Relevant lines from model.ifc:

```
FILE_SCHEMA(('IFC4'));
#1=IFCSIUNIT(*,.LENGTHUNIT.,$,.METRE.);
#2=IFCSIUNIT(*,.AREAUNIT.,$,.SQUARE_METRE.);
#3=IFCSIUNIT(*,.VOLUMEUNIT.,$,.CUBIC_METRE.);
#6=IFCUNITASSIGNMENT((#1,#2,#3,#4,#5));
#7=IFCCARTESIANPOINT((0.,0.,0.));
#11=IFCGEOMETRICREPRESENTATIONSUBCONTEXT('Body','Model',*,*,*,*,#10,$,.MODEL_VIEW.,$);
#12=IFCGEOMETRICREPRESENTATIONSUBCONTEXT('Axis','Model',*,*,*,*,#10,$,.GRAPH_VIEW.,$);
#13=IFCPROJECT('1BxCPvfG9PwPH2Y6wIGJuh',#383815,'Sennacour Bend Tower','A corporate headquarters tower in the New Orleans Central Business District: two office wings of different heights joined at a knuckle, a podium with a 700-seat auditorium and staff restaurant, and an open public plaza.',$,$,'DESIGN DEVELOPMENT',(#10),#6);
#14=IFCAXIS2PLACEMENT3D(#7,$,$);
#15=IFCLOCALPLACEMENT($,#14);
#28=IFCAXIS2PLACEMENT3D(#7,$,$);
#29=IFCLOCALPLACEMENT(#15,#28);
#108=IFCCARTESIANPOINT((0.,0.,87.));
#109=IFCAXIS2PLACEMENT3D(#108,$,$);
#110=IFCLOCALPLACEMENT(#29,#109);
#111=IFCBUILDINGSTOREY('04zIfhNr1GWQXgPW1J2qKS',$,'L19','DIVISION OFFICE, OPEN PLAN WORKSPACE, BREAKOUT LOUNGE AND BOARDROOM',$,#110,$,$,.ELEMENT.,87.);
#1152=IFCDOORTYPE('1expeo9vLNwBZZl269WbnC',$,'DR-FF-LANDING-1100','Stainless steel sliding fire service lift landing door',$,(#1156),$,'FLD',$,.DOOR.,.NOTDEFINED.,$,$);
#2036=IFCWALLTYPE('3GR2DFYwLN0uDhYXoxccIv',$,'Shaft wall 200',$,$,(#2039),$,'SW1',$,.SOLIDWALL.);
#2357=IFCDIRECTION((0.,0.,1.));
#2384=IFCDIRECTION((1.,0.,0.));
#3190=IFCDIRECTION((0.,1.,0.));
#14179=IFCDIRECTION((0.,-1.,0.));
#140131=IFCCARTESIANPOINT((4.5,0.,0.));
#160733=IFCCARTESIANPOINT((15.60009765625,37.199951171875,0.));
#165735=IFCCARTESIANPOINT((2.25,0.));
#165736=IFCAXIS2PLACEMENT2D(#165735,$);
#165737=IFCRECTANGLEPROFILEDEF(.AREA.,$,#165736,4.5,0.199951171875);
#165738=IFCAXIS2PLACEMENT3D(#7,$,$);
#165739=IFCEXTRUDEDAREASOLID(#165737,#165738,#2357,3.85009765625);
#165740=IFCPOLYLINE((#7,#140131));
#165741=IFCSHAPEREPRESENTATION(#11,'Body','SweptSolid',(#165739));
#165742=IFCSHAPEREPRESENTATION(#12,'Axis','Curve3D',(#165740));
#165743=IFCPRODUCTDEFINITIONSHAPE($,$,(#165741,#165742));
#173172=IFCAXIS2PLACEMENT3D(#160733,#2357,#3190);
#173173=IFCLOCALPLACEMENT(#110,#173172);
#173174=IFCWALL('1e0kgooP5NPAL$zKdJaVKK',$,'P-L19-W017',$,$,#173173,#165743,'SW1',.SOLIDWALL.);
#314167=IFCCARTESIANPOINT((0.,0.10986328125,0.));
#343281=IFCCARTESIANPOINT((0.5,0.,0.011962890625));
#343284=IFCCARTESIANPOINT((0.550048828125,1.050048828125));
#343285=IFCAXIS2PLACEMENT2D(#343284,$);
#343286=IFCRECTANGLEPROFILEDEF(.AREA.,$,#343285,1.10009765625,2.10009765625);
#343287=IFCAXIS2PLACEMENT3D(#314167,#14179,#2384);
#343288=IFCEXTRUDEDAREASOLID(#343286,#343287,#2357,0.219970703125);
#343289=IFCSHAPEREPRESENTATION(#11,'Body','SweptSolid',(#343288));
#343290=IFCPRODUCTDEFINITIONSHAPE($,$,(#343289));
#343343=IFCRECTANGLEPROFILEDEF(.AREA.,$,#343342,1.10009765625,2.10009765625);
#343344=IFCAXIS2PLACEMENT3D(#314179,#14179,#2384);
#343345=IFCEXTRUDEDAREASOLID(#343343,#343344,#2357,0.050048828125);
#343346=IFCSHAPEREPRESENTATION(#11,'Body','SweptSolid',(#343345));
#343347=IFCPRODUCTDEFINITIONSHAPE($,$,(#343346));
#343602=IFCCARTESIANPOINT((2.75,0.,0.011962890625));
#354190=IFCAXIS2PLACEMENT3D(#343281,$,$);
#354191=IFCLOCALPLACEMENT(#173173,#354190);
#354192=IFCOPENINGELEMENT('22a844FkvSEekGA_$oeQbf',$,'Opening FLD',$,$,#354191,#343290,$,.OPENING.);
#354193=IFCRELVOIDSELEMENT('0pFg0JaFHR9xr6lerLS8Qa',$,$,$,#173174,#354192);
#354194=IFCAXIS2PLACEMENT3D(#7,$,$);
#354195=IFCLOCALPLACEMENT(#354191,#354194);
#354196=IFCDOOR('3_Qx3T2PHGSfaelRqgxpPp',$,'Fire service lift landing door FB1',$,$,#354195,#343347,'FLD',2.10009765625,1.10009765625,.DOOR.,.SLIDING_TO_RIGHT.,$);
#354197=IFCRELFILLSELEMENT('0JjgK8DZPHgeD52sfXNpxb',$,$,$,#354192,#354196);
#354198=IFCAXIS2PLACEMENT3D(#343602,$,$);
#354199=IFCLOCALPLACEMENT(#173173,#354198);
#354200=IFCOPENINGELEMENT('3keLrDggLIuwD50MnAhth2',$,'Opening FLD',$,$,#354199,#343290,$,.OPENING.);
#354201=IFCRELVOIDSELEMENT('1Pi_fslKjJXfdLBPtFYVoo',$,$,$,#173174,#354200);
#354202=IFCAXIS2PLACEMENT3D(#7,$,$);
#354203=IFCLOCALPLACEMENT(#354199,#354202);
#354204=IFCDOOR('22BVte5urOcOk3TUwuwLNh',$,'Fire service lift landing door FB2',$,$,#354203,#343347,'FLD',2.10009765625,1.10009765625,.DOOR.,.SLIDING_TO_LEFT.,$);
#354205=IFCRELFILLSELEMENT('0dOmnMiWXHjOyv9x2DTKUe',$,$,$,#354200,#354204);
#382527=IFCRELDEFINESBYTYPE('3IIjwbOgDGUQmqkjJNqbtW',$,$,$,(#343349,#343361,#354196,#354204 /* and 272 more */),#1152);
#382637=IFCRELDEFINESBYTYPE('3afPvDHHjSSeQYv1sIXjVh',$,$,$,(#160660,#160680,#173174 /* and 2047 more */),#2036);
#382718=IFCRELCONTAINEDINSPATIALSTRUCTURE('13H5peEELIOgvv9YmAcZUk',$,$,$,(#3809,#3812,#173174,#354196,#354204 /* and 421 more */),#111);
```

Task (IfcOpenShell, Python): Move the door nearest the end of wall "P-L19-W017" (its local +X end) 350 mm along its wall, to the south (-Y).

```python
import ifcopenshell
import ifcopenshell.api.geometry
import ifcopenshell.util.placement
import ifcopenshell.util.unit

model = ifcopenshell.open("model.ifc")
unit_scale = ifcopenshell.util.unit.calculate_unit_scale(model)

door = model.by_guid("22BVte5urOcOk3TUwuwLNh")
opening = door.FillsVoids[0].RelatingOpeningElement
wall = opening.VoidsElements[0].RelatingBuildingElement

wall_matrix = ifcopenshell.util.placement.get_local_placement(wall.ObjectPlacement)
shift = wall_matrix[:3, 0] * -0.35 / unit_scale
before = ifcopenshell.util.placement.get_local_placement(door.ObjectPlacement)[:3, 3].copy()

# The door is placed relative to its opening, so it follows when the opening moves.
matrix = ifcopenshell.util.placement.get_local_placement(opening.ObjectPlacement)
matrix[:3, 3] += shift
ifcopenshell.api.geometry.edit_object_placement(
    model, product=opening, matrix=matrix, is_si=False, should_transform_children=True
)

after = ifcopenshell.util.placement.get_local_placement(door.ObjectPlacement)[:3, 3]
print("door moved by", (after - before).round(3) + 0.0)

model.write("model-out.ifc")
```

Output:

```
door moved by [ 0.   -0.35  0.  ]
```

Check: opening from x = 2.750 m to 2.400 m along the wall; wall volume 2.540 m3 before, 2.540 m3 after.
